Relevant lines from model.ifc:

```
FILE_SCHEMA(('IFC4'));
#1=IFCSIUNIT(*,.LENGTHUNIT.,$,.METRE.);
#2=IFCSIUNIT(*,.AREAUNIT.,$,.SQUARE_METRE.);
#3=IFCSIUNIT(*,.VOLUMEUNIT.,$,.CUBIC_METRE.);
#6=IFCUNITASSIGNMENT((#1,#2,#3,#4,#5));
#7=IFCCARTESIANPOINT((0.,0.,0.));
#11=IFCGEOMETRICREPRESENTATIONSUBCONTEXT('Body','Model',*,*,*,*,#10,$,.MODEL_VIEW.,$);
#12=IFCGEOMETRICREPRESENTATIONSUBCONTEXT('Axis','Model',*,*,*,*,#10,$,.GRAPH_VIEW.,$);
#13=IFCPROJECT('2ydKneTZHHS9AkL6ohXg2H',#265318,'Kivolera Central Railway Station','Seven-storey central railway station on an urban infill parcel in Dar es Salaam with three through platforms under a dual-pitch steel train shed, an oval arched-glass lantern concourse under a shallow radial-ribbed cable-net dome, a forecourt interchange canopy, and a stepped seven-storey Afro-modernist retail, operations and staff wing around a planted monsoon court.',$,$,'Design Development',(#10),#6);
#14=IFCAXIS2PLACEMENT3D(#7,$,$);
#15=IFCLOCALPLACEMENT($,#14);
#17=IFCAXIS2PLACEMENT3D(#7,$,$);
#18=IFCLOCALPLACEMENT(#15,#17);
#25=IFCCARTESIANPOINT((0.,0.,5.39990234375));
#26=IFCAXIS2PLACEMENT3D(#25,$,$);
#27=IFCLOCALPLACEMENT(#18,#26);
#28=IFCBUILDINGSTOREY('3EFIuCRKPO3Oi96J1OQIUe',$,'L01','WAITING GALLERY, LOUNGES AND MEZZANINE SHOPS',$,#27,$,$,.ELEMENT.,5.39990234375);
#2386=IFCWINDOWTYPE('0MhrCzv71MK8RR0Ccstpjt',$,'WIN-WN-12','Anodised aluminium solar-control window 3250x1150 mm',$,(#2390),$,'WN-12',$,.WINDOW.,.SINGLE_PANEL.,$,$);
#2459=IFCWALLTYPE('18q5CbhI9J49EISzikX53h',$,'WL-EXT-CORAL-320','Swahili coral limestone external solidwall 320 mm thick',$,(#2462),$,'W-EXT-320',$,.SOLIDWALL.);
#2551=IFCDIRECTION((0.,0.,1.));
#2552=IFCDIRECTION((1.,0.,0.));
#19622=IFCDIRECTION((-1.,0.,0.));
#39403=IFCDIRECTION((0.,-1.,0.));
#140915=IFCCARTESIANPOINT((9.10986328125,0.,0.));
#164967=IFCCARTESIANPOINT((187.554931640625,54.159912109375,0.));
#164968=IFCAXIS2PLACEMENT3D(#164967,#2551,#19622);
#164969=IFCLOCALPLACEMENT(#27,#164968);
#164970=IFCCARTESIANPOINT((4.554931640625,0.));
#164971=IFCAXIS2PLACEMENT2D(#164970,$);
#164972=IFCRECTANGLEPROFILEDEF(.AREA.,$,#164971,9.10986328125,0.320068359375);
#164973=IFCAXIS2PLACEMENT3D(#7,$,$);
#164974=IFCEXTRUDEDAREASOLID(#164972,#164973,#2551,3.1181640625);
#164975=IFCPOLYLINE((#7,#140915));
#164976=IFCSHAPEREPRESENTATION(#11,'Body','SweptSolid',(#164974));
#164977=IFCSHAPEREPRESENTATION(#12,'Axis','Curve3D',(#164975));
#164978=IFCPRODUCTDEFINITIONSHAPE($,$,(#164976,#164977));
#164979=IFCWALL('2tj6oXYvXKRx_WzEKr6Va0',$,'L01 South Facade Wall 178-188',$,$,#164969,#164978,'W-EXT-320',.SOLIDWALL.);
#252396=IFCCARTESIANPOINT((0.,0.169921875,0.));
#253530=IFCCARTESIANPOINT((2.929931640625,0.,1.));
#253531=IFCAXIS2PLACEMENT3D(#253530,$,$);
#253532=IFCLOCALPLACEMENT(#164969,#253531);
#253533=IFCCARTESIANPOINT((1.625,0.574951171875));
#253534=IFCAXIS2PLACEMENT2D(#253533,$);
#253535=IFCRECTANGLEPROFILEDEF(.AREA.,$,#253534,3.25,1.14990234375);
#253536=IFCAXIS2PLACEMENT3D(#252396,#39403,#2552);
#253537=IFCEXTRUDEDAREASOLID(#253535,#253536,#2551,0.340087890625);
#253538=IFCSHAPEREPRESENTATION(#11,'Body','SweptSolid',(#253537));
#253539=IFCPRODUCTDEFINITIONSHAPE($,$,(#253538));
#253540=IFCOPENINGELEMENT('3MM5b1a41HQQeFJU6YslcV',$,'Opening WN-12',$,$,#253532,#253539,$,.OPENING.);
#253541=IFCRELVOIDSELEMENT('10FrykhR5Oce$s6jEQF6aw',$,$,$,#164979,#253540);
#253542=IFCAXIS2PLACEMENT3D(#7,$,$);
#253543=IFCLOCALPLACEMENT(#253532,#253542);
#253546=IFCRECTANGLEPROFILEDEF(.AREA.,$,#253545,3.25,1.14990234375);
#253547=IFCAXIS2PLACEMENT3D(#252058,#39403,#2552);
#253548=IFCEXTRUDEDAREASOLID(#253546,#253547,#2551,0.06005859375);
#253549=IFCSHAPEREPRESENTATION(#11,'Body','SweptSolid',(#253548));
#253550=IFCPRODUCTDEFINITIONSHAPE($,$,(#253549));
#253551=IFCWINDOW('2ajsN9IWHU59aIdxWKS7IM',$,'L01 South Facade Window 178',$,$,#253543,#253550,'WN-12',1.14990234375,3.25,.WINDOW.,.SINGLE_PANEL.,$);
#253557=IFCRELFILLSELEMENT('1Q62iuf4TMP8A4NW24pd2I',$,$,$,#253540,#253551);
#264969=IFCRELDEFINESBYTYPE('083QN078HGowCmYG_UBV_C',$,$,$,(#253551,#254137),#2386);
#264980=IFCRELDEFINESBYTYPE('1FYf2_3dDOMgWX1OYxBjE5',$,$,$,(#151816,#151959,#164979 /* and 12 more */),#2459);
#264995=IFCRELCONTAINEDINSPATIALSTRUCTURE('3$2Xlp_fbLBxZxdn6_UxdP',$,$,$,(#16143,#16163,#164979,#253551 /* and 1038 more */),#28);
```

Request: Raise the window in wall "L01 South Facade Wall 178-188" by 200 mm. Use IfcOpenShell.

```python
import numpy as np
import ifcopenshell
import ifcopenshell.api.geometry
import ifcopenshell.util.placement
import ifcopenshell.util.unit

model = ifcopenshell.open("model.ifc")
unit_scale = ifcopenshell.util.unit.calculate_unit_scale(model)

window = model.by_id(253551)
opening = window.FillsVoids[0].RelatingOpeningElement
dz = 0.2 / unit_scale

shift = np.array([0.0, 0.0, dz])
# The window is placed relative to its opening, so it follows when the opening moves.
matrix = ifcopenshell.util.placement.get_local_placement(opening.ObjectPlacement)
matrix[:3, 3] += shift
ifcopenshell.api.geometry.edit_object_placement(
    model, product=opening, matrix=matrix, is_si=False, should_transform_children=True
)

print(f"moved by {dz * unit_scale:+.3f} m")

model.write("model_edited.ifc")
```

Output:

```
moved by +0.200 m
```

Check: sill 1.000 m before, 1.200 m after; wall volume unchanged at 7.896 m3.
